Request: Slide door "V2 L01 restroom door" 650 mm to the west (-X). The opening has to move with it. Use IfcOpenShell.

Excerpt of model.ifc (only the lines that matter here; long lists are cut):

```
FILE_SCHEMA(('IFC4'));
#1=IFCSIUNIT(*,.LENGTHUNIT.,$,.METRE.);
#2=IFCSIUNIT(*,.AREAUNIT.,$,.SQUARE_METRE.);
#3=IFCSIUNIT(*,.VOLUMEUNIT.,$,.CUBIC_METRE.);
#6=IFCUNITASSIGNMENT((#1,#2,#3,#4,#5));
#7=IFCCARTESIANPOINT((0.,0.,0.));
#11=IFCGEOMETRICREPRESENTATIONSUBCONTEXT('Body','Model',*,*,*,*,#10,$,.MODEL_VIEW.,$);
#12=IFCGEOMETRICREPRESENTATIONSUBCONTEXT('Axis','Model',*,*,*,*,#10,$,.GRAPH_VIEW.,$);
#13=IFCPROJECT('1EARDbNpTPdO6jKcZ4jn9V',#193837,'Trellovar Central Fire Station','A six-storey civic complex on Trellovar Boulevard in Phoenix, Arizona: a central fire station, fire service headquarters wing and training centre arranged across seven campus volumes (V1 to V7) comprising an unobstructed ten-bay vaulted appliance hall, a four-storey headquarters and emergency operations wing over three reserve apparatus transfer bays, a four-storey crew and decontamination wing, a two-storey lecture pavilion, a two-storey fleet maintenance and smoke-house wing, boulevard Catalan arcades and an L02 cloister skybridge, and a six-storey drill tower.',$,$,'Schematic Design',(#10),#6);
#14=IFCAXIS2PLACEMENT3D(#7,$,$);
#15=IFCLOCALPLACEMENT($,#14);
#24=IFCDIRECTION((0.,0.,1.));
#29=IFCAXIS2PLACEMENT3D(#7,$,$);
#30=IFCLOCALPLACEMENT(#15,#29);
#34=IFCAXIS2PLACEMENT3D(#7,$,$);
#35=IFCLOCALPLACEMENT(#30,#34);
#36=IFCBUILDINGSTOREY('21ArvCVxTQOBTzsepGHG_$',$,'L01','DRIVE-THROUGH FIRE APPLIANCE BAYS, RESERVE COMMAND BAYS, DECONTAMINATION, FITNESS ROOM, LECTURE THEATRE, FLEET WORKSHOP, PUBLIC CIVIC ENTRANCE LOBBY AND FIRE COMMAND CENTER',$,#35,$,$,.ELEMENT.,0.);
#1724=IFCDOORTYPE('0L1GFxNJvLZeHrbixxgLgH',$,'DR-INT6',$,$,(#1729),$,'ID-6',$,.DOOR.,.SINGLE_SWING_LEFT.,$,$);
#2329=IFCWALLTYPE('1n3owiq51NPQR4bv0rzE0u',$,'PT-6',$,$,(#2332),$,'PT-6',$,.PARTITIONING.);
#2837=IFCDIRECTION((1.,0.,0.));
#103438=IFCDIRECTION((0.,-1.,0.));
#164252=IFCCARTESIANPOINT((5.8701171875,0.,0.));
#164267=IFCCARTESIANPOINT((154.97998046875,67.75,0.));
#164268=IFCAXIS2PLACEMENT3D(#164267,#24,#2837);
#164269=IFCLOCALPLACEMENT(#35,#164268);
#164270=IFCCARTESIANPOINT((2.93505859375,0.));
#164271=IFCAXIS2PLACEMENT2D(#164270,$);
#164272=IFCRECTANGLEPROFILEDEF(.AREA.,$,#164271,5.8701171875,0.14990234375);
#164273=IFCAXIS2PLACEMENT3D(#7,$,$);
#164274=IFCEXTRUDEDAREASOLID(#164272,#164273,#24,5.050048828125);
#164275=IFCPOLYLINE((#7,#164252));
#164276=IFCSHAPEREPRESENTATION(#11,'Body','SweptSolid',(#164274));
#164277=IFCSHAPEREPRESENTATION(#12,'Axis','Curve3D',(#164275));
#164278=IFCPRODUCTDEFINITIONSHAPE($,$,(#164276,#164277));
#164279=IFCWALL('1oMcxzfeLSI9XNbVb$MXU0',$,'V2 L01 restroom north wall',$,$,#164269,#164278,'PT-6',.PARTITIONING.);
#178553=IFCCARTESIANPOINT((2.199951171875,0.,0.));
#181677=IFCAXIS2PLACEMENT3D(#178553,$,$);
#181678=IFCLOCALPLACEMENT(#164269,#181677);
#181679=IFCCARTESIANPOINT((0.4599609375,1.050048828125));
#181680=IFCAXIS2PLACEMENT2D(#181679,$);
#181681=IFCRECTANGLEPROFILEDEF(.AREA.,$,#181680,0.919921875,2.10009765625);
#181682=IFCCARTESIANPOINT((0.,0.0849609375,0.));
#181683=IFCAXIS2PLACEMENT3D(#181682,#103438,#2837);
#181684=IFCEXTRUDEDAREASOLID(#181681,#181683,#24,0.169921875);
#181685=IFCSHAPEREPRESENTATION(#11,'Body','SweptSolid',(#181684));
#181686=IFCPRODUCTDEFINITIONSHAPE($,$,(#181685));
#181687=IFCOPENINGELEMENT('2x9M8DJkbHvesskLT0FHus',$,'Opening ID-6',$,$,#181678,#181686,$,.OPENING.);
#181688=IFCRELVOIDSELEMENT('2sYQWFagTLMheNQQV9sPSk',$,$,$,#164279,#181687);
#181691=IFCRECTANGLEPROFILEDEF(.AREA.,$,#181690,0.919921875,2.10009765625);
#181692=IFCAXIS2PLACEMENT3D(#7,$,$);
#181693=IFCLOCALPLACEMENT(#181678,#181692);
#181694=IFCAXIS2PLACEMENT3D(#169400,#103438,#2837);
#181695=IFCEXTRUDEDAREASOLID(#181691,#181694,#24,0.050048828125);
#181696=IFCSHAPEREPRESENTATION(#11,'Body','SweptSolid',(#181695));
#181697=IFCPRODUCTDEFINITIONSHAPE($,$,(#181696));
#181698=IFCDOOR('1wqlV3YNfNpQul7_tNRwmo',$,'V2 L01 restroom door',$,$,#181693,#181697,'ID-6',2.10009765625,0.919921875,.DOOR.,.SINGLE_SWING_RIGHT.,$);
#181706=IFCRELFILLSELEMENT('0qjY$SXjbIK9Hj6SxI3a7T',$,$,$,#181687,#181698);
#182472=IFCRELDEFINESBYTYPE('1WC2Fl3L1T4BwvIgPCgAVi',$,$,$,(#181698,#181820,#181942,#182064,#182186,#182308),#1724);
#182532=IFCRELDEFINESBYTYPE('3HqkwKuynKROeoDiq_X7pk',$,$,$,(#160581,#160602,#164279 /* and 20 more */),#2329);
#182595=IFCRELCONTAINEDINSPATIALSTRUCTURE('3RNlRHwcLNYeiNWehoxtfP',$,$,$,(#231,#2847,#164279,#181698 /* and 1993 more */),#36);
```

```python
import ifcopenshell
import ifcopenshell.api.geometry
import ifcopenshell.util.placement
import ifcopenshell.util.unit

model = ifcopenshell.open("model.ifc")
unit_scale = ifcopenshell.util.unit.calculate_unit_scale(model)

door = model.by_guid("1wqlV3YNfNpQul7_tNRwmo")
opening = door.FillsVoids[0].RelatingOpeningElement
wall = opening.VoidsElements[0].RelatingBuildingElement

wall_matrix = ifcopenshell.util.placement.get_local_placement(wall.ObjectPlacement)
shift = wall_matrix[:3, 0] * -0.65 / unit_scale
before = ifcopenshell.util.placement.get_local_placement(door.ObjectPlacement)[:3, 3].copy()

# The door is placed relative to its opening, so it follows when the opening moves.
matrix = ifcopenshell.util.placement.get_local_placement(opening.ObjectPlacement)
matrix[:3, 3] += shift
ifcopenshell.api.geometry.edit_object_placement(
    model, product=opening, matrix=matrix, is_si=False, should_transform_children=True
)

after = ifcopenshell.util.placement.get_local_placement(door.ObjectPlacement)[:3, 3]
print("door moved by", (after - before).round(3) + 0.0)

model.write("model-out.ifc")
```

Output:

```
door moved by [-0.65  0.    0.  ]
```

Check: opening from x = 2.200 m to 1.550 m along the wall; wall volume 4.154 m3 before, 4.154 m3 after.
